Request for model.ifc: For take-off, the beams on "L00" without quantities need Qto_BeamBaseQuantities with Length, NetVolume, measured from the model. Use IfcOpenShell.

First a look at what the model holds.

```python
import ifcopenshell
import ifcopenshell.util.element
import ifcopenshell.util.unit

model = ifcopenshell.open("model.ifc")
print(model.schema)
for unit_type in ("LENGTHUNIT", "AREAUNIT", "VOLUMEUNIT"):
    print(unit_type, ifcopenshell.util.unit.calculate_unit_scale(model, unit_type))
storey = next(s for s in model.by_type("IfcBuildingStorey") if s.Name == "L00")
beams = [e for e in ifcopenshell.util.element.get_decomposition(storey) if e.is_a("IfcBeam")]
for e in sorted(beams, key=lambda e: e.id()):
    print(e.id(), e.is_a(), e.Name, list(ifcopenshell.util.element.get_psets(e, qtos_only=True)), sep=" | ")
```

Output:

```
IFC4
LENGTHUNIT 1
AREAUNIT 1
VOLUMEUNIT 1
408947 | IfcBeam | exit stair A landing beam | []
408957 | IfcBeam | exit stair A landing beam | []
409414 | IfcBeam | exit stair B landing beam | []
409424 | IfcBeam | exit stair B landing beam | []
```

```python
import ifcopenshell
import ifcopenshell.api.pset
import ifcopenshell.geom
import ifcopenshell.util.element
import ifcopenshell.util.shape
import ifcopenshell.util.unit

model = ifcopenshell.open("model.ifc")
unit_scale = ifcopenshell.util.unit.calculate_unit_scale(model)
volume_scale = ifcopenshell.util.unit.calculate_unit_scale(model, "VOLUMEUNIT")
settings = ifcopenshell.geom.settings()

storey = next(s for s in model.by_type("IfcBuildingStorey") if s.Name == "L00")
beams = [e for e in ifcopenshell.util.element.get_decomposition(storey) if e.is_a("IfcBeam")]

for e in sorted(beams, key=lambda e: e.id()):
    if ifcopenshell.util.element.get_psets(e, qtos_only=True, should_inherit=False):
        continue
    # Geometry comes back in metres, in the element's own axes.
    shape = ifcopenshell.geom.create_shape(settings, e)
    values = {
        "Length": ifcopenshell.util.shape.get_max_xyz(shape.geometry) / unit_scale,
        "NetVolume": ifcopenshell.util.shape.get_volume(shape.geometry) / volume_scale,
    }
    qto = ifcopenshell.api.pset.add_qto(model, product=e, name="Qto_BeamBaseQuantities")
    ifcopenshell.api.pset.edit_qto(model, qto=qto, properties=values)
    print(e.id(), {k: round(v, 3) for k, v in values.items()})

model.write("model_v2.ifc")
```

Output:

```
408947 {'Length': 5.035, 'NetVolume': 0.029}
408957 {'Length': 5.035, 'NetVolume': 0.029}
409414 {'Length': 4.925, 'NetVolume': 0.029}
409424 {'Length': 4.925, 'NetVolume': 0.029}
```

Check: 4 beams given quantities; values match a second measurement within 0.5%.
